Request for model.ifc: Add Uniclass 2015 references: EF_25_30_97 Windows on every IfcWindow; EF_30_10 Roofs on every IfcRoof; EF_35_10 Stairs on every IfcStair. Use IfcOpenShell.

First a look at what the model holds.

```python
import ifcopenshell

model = ifcopenshell.open("model.ifc")
print(model.schema)
print("classifications:", [c.Name for c in model.by_type("IfcClassification")])
for ifc_class in ("IfcDoor", "IfcRoof", "IfcStair", "IfcWall", "IfcWindow"):
    print(ifc_class, len(model.by_type(ifc_class)))
```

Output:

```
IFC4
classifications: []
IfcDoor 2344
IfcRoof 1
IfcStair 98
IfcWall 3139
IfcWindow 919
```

```python
import ifcopenshell
import ifcopenshell.api.classification

model = ifcopenshell.open("model.ifc")

system = ifcopenshell.api.classification.add_classification(model, classification="Uniclass 2015")

codes = {
    "IfcWindow": ("EF_25_30_97", "Windows"),
    "IfcRoof": ("EF_30_10", "Roofs"),
    "IfcStair": ("EF_35_10", "Stairs"),
}
for ifc_class, (code, name) in codes.items():
    products = model.by_type(ifc_class)
    ifcopenshell.api.classification.add_reference(
        model, products=products, classification=system, identification=code, name=name
    )
    print(code, len(products))

model.write("model_v2.ifc")
```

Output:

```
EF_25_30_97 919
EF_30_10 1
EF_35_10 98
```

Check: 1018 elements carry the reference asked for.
